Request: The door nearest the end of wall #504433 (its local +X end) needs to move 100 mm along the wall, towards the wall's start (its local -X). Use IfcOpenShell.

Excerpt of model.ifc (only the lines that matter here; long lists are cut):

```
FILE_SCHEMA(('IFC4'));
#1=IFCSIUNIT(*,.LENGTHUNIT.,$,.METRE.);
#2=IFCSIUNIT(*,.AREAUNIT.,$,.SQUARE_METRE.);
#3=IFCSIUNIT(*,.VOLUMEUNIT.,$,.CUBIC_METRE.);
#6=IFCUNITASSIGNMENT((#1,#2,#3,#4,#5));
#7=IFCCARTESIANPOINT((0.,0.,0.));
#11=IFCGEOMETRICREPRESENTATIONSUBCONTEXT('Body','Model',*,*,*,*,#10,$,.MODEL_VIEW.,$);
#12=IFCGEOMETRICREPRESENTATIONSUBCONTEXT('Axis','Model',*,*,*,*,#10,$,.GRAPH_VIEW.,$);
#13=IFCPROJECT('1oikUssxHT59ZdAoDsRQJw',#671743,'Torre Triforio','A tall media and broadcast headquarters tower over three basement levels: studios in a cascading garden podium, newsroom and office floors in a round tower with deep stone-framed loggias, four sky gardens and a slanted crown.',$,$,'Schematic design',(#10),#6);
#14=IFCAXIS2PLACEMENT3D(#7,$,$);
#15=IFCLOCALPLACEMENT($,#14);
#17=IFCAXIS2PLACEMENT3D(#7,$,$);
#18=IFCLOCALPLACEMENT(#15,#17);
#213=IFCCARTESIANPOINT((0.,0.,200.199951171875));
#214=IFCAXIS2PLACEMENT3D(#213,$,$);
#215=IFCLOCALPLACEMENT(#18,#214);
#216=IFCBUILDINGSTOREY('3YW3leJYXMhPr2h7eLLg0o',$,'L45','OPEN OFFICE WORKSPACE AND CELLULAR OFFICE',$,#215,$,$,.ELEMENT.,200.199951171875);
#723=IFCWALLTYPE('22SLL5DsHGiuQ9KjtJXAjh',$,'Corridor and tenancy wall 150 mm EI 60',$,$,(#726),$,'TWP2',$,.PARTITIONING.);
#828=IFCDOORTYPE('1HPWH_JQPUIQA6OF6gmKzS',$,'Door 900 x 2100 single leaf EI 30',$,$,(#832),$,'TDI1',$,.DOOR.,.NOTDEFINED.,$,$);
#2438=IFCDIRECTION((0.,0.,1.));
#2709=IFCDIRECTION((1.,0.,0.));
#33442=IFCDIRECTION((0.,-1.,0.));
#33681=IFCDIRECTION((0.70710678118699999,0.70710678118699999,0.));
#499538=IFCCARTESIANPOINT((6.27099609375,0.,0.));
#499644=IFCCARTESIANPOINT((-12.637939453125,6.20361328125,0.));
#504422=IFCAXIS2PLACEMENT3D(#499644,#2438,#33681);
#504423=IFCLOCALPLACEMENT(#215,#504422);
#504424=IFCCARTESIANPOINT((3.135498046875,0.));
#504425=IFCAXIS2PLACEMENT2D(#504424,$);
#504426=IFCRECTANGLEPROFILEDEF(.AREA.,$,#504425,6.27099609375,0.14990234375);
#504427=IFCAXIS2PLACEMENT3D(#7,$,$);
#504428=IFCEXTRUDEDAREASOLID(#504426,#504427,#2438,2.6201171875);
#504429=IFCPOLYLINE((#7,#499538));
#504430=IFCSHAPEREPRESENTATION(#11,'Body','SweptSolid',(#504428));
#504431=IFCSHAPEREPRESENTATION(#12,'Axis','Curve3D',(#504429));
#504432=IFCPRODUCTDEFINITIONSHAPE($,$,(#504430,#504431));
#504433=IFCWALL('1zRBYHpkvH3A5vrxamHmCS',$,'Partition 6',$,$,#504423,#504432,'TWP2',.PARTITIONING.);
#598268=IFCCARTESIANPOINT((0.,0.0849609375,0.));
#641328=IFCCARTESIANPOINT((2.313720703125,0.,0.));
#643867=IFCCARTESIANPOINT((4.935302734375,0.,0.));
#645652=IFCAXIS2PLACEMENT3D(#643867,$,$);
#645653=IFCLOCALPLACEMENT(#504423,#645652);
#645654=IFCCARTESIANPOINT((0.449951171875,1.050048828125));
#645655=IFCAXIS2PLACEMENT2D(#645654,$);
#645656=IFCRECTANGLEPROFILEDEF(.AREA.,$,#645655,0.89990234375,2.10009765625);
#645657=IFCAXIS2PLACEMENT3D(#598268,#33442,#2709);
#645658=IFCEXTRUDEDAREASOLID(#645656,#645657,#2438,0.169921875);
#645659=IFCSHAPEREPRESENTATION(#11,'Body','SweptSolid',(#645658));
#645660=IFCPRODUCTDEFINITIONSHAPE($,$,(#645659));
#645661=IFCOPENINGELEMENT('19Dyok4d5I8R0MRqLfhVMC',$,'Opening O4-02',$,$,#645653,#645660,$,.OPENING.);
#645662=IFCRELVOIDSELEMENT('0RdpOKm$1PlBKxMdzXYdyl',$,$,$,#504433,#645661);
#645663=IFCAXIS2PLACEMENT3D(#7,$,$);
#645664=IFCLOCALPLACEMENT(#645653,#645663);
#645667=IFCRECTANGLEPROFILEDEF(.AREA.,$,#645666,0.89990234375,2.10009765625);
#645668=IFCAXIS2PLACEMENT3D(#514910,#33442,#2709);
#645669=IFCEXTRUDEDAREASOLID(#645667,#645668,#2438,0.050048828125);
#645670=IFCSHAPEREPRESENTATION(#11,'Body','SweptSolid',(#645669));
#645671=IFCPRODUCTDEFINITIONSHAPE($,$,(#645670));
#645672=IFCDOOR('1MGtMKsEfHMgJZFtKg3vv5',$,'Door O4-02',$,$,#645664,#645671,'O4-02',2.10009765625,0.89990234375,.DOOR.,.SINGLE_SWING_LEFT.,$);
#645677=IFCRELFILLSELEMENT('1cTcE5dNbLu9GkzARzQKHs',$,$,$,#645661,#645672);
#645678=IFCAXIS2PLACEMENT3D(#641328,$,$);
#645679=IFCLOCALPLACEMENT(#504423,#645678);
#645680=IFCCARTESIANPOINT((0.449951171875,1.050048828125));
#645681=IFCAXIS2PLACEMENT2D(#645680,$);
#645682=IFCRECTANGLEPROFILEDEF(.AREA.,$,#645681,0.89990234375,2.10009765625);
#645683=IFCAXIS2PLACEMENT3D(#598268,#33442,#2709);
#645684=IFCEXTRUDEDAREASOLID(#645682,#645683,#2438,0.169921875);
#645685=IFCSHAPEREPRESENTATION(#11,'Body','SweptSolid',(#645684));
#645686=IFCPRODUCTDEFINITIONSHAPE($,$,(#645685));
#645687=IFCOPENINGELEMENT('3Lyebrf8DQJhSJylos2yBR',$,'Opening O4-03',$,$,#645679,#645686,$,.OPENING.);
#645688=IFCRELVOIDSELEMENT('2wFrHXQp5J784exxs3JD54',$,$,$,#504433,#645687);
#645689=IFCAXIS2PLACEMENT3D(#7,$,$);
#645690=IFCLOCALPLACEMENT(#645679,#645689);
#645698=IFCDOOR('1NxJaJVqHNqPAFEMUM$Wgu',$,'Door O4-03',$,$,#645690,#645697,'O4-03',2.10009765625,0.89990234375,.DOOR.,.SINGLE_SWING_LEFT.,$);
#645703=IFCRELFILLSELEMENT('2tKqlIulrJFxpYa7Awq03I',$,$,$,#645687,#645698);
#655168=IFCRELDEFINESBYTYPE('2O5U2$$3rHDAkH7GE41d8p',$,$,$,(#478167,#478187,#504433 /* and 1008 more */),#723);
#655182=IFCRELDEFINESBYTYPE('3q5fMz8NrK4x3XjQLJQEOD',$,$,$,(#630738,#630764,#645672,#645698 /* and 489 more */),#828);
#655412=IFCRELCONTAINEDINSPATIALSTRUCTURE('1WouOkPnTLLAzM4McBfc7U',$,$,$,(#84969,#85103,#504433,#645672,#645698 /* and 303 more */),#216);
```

```python
import ifcopenshell
import ifcopenshell.api.geometry
import ifcopenshell.util.placement

model = ifcopenshell.open("model.ifc")

door = model.by_guid("1MGtMKsEfHMgJZFtKg3vv5")
opening = door.FillsVoids[0].RelatingOpeningElement
wall = opening.VoidsElements[0].RelatingBuildingElement

wall_matrix = ifcopenshell.util.placement.get_local_placement(wall.ObjectPlacement)
shift = wall_matrix[:3, 0] * -0.1
before = ifcopenshell.util.placement.get_local_placement(door.ObjectPlacement)[:3, 3].copy()

# The door is placed relative to its opening, so it follows when the opening moves.
matrix = ifcopenshell.util.placement.get_local_placement(opening.ObjectPlacement)
matrix[:3, 3] += shift
ifcopenshell.api.geometry.edit_object_placement(
    model, product=opening, matrix=matrix, is_si=False, should_transform_children=True
)

after = ifcopenshell.util.placement.get_local_placement(door.ObjectPlacement)[:3, 3]
print("door moved by", (after - before).round(3) + 0.0)

model.write("model_rev.ifc")
```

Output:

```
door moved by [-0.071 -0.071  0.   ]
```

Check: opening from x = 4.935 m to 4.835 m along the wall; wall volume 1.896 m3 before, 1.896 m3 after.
